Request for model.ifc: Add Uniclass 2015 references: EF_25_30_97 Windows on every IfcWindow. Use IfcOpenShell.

First a look at what the model holds.

```python
import ifcopenshell

model = ifcopenshell.open("model.ifc")
print(model.schema)
print("classifications:", [c.Name for c in model.by_type("IfcClassification")])
for ifc_class in ("IfcDoor", "IfcRoof", "IfcStair", "IfcWall", "IfcWindow"):
    print(ifc_class, len(model.by_type(ifc_class)))
```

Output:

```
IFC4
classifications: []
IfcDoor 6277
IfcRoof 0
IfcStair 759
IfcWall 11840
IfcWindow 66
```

```python
import ifcopenshell
import ifcopenshell.api.classification

model = ifcopenshell.open("model.ifc")

system = ifcopenshell.api.classification.add_classification(model, classification="Uniclass 2015")

codes = {
    "IfcWindow": ("EF_25_30_97", "Windows"),
}
for ifc_class, (code, name) in codes.items():
    products = model.by_type(ifc_class)
    ifcopenshell.api.classification.add_reference(
        model, products=products, classification=system, identification=code, name=name
    )
    print(code, len(products))

model.write("model_updated.ifc")
```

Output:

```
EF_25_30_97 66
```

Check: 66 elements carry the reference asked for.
